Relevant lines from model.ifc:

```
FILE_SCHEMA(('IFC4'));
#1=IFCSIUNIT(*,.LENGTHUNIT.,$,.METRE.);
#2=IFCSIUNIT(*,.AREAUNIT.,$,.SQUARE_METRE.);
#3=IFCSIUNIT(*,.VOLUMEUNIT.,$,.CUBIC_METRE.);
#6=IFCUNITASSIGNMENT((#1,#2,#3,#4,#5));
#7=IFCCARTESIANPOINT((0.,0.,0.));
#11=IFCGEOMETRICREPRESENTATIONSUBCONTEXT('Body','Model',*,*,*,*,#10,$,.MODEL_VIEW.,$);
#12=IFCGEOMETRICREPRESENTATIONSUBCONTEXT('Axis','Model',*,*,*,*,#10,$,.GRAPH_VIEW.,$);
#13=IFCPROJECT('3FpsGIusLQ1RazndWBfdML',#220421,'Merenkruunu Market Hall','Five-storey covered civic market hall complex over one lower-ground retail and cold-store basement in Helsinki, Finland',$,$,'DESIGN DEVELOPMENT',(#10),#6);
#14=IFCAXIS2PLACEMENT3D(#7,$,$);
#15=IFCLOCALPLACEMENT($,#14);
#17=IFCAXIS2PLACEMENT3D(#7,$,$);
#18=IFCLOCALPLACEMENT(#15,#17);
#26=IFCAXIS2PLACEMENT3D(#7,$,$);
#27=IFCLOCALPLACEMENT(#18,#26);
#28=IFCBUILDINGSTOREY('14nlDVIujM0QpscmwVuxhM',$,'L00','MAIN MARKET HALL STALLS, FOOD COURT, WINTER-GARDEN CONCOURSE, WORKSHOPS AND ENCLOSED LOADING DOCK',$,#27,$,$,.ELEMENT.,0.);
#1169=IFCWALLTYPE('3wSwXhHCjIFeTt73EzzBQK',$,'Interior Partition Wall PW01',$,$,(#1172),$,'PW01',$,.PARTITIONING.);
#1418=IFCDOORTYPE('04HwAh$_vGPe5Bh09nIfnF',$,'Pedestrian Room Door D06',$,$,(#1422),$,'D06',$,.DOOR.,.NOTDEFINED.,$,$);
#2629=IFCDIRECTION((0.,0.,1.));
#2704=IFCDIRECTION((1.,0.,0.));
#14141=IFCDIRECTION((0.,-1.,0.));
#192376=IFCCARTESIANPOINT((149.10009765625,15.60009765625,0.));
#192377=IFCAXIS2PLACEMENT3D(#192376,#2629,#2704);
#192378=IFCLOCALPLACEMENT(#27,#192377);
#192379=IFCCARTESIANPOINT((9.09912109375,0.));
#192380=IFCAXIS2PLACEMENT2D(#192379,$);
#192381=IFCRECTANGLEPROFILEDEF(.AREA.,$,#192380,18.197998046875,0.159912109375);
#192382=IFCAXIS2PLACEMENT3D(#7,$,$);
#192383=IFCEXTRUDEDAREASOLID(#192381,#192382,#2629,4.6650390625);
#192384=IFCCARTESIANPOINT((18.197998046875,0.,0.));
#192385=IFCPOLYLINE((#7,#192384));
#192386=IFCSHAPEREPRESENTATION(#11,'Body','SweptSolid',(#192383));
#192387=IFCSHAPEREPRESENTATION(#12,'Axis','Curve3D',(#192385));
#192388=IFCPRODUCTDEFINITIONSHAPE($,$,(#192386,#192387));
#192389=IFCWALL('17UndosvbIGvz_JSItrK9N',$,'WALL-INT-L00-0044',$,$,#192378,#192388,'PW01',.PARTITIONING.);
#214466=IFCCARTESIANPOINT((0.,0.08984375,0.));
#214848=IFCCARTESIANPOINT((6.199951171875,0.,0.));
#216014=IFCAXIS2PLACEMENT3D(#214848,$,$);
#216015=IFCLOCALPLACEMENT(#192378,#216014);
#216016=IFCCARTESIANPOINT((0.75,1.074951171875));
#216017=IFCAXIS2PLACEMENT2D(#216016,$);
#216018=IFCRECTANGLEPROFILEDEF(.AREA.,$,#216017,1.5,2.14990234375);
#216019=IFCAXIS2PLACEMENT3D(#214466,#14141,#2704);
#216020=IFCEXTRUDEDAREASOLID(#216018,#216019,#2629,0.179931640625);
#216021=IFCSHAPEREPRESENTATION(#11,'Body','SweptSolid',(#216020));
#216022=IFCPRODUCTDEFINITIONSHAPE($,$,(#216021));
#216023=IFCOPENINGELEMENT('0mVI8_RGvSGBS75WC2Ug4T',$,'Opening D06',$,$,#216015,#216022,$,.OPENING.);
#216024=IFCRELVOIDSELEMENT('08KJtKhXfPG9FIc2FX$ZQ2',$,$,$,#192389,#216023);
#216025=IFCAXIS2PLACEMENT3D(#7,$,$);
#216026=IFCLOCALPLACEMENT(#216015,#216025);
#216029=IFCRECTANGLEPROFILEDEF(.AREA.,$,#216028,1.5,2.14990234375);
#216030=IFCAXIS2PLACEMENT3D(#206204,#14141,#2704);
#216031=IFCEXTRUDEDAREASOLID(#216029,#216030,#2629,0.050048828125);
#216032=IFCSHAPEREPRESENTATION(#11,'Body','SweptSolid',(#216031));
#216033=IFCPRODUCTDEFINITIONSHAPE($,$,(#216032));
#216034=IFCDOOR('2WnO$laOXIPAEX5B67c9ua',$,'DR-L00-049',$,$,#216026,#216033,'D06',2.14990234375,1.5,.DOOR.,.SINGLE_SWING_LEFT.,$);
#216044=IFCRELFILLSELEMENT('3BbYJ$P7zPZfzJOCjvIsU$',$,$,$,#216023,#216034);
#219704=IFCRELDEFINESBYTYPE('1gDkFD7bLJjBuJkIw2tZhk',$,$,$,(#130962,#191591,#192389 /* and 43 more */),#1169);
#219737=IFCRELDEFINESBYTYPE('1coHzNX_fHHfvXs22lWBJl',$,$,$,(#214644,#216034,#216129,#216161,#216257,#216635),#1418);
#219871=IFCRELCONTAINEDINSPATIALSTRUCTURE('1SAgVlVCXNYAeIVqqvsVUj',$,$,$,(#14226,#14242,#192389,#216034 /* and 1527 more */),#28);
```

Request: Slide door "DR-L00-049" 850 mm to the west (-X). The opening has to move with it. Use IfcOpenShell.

```python
import ifcopenshell
import ifcopenshell.api.geometry
import ifcopenshell.util.placement

model = ifcopenshell.open("model.ifc")

door = model.by_id(216034)
opening = door.FillsVoids[0].RelatingOpeningElement
wall = opening.VoidsElements[0].RelatingBuildingElement

wall_matrix = ifcopenshell.util.placement.get_local_placement(wall.ObjectPlacement)
shift = wall_matrix[:3, 0] * -0.85
before = ifcopenshell.util.placement.get_local_placement(door.ObjectPlacement)[:3, 3].copy()

# The door is placed relative to its opening, so it follows when the opening moves.
matrix = ifcopenshell.util.placement.get_local_placement(opening.ObjectPlacement)
matrix[:3, 3] += shift
ifcopenshell.api.geometry.edit_object_placement(
    model, product=opening, matrix=matrix, is_si=False, should_transform_children=True
)

after = ifcopenshell.util.placement.get_local_placement(door.ObjectPlacement)[:3, 3]
print("door moved by", (after - before).round(3) + 0.0)

model.write("model_edited.ifc")
```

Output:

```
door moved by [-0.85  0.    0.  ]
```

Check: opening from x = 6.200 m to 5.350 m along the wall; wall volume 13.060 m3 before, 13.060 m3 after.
